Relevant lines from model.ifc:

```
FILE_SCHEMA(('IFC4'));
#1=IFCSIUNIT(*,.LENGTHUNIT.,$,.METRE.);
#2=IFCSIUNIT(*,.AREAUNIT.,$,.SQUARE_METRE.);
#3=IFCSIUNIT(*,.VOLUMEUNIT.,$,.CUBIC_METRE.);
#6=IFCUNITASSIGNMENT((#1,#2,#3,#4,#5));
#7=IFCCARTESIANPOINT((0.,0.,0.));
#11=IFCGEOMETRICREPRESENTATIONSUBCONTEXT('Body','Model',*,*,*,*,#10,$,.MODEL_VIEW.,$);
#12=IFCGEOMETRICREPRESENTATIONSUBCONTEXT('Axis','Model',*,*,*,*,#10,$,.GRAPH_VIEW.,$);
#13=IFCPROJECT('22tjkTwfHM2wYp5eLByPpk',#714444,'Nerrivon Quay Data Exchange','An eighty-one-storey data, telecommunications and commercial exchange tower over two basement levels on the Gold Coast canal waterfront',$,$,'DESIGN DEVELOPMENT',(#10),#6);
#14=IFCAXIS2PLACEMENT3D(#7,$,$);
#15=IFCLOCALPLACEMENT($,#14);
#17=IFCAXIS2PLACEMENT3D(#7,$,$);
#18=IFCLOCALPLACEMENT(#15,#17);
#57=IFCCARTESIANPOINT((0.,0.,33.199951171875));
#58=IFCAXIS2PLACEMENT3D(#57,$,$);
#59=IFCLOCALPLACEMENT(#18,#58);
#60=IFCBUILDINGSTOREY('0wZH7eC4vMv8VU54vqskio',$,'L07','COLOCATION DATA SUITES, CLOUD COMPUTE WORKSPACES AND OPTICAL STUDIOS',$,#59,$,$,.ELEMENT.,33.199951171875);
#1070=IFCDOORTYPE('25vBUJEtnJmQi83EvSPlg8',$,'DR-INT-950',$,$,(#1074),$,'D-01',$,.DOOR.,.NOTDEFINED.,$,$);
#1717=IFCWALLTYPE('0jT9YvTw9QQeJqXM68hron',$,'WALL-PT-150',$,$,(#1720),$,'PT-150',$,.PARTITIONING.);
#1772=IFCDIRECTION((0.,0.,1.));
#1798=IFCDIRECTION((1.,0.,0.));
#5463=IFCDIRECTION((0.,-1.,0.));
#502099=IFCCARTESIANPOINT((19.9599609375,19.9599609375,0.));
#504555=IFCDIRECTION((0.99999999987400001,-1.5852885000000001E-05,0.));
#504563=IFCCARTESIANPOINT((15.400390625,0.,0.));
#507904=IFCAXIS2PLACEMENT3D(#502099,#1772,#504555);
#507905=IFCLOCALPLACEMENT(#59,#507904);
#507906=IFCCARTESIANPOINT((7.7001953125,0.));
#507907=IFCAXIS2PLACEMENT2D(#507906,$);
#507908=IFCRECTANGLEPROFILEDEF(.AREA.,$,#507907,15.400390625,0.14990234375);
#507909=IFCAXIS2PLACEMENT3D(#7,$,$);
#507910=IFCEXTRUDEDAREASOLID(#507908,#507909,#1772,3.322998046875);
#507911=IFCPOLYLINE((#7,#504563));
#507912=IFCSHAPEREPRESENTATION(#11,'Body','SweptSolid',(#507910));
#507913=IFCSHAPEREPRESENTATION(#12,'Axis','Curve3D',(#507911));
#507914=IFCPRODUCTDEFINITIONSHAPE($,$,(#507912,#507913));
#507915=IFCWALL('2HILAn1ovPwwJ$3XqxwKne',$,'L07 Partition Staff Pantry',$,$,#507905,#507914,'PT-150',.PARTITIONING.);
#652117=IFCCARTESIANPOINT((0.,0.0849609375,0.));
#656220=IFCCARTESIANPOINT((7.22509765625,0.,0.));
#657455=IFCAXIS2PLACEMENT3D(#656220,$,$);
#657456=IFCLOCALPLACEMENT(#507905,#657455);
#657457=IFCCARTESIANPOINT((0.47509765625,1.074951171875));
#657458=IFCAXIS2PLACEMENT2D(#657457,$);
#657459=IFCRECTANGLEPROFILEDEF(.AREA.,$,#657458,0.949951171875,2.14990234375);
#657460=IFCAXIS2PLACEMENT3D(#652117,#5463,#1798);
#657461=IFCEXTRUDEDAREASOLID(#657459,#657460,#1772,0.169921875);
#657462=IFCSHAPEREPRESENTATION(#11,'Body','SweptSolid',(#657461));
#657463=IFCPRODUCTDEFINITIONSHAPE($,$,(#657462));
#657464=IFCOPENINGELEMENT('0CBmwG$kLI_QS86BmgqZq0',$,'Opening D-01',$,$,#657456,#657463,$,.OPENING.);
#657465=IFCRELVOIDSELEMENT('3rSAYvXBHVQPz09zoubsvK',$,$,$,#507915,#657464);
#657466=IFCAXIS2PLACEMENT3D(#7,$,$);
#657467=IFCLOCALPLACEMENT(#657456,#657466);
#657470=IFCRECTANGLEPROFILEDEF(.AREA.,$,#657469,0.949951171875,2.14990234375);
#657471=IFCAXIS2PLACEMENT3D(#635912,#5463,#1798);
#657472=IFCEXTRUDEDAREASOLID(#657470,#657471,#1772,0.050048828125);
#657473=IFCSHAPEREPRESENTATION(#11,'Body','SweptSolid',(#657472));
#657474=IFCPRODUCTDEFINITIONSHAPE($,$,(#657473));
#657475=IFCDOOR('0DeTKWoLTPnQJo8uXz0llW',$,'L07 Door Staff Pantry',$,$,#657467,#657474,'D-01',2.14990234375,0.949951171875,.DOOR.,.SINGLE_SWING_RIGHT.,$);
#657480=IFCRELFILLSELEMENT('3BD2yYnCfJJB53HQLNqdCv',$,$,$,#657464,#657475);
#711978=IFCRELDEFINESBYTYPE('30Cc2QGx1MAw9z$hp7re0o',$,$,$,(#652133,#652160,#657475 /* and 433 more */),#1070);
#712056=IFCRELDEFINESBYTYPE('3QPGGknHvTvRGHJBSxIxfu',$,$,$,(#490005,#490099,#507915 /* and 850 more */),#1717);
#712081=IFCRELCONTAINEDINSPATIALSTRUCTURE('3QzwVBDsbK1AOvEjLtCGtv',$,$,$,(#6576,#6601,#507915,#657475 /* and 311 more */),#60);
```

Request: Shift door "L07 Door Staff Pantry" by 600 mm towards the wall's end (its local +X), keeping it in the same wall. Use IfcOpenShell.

```python
import ifcopenshell
import ifcopenshell.api.geometry
import ifcopenshell.util.placement

model = ifcopenshell.open("model.ifc")

door = model.by_guid("0DeTKWoLTPnQJo8uXz0llW")
opening = door.FillsVoids[0].RelatingOpeningElement
wall = opening.VoidsElements[0].RelatingBuildingElement

wall_matrix = ifcopenshell.util.placement.get_local_placement(wall.ObjectPlacement)
shift = wall_matrix[:3, 0] * 0.6
before = ifcopenshell.util.placement.get_local_placement(door.ObjectPlacement)[:3, 3].copy()

# The door is placed relative to its opening, so it follows when the opening moves.
matrix = ifcopenshell.util.placement.get_local_placement(opening.ObjectPlacement)
matrix[:3, 3] += shift
ifcopenshell.api.geometry.edit_object_placement(
    model, product=opening, matrix=matrix, is_si=False, should_transform_children=True
)

after = ifcopenshell.util.placement.get_local_placement(door.ObjectPlacement)[:3, 3]
print("door moved by", (after - before).round(3) + 0.0)

model.write("model_rev.ifc")
```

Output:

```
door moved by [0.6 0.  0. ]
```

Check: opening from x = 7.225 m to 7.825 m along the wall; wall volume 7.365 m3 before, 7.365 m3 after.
